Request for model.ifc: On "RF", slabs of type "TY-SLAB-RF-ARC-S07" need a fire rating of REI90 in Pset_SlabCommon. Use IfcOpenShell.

First a look at what the model holds.

```python
import ifcopenshell
import ifcopenshell.util.element

model = ifcopenshell.open("model.ifc")
print(model.schema)
storey = next(s for s in model.by_type("IfcBuildingStorey") if s.Name == "RF")
slabs = [e for e in ifcopenshell.util.element.get_decomposition(storey) if e.is_a("IfcSlab")]
seen = {}
for e in slabs:
    element_type = ifcopenshell.util.element.get_type(e)
    key = (element_type.Name if element_type != e and element_type else None, ifcopenshell.util.element.get_pset(e, "Pset_SlabCommon", "FireRating"))
    seen[key] = seen.get(key, 0) + 1
for (name, value), count in sorted(seen.items(), key=str):
    print(count, "x", name, "|", value)
```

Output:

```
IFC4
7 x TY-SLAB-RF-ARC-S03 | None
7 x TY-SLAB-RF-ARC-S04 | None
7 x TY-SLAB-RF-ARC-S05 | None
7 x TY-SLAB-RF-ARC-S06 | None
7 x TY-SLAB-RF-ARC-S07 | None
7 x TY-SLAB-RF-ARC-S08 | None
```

```python
import ifcopenshell
import ifcopenshell.api.pset
import ifcopenshell.util.element

model = ifcopenshell.open("model.ifc")

storey = next(s for s in model.by_type("IfcBuildingStorey") if s.Name == "RF")
slabs = [e for e in ifcopenshell.util.element.get_decomposition(storey) if e.is_a("IfcSlab")]

count = 0
for e in slabs:
    element_type = ifcopenshell.util.element.get_type(e)
    if element_type in (None, e) or element_type.Name != "TY-SLAB-RF-ARC-S07":
        continue
    # add_pset returns the element's existing set when there is one.
    pset = ifcopenshell.api.pset.add_pset(model, product=e, name="Pset_SlabCommon")
    ifcopenshell.api.pset.edit_pset(model, pset=pset, properties={"FireRating": "REI90"})
    count += 1

print(count, "slabs updated")

model.write("model_rev.ifc")
```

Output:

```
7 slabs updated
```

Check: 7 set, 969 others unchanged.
